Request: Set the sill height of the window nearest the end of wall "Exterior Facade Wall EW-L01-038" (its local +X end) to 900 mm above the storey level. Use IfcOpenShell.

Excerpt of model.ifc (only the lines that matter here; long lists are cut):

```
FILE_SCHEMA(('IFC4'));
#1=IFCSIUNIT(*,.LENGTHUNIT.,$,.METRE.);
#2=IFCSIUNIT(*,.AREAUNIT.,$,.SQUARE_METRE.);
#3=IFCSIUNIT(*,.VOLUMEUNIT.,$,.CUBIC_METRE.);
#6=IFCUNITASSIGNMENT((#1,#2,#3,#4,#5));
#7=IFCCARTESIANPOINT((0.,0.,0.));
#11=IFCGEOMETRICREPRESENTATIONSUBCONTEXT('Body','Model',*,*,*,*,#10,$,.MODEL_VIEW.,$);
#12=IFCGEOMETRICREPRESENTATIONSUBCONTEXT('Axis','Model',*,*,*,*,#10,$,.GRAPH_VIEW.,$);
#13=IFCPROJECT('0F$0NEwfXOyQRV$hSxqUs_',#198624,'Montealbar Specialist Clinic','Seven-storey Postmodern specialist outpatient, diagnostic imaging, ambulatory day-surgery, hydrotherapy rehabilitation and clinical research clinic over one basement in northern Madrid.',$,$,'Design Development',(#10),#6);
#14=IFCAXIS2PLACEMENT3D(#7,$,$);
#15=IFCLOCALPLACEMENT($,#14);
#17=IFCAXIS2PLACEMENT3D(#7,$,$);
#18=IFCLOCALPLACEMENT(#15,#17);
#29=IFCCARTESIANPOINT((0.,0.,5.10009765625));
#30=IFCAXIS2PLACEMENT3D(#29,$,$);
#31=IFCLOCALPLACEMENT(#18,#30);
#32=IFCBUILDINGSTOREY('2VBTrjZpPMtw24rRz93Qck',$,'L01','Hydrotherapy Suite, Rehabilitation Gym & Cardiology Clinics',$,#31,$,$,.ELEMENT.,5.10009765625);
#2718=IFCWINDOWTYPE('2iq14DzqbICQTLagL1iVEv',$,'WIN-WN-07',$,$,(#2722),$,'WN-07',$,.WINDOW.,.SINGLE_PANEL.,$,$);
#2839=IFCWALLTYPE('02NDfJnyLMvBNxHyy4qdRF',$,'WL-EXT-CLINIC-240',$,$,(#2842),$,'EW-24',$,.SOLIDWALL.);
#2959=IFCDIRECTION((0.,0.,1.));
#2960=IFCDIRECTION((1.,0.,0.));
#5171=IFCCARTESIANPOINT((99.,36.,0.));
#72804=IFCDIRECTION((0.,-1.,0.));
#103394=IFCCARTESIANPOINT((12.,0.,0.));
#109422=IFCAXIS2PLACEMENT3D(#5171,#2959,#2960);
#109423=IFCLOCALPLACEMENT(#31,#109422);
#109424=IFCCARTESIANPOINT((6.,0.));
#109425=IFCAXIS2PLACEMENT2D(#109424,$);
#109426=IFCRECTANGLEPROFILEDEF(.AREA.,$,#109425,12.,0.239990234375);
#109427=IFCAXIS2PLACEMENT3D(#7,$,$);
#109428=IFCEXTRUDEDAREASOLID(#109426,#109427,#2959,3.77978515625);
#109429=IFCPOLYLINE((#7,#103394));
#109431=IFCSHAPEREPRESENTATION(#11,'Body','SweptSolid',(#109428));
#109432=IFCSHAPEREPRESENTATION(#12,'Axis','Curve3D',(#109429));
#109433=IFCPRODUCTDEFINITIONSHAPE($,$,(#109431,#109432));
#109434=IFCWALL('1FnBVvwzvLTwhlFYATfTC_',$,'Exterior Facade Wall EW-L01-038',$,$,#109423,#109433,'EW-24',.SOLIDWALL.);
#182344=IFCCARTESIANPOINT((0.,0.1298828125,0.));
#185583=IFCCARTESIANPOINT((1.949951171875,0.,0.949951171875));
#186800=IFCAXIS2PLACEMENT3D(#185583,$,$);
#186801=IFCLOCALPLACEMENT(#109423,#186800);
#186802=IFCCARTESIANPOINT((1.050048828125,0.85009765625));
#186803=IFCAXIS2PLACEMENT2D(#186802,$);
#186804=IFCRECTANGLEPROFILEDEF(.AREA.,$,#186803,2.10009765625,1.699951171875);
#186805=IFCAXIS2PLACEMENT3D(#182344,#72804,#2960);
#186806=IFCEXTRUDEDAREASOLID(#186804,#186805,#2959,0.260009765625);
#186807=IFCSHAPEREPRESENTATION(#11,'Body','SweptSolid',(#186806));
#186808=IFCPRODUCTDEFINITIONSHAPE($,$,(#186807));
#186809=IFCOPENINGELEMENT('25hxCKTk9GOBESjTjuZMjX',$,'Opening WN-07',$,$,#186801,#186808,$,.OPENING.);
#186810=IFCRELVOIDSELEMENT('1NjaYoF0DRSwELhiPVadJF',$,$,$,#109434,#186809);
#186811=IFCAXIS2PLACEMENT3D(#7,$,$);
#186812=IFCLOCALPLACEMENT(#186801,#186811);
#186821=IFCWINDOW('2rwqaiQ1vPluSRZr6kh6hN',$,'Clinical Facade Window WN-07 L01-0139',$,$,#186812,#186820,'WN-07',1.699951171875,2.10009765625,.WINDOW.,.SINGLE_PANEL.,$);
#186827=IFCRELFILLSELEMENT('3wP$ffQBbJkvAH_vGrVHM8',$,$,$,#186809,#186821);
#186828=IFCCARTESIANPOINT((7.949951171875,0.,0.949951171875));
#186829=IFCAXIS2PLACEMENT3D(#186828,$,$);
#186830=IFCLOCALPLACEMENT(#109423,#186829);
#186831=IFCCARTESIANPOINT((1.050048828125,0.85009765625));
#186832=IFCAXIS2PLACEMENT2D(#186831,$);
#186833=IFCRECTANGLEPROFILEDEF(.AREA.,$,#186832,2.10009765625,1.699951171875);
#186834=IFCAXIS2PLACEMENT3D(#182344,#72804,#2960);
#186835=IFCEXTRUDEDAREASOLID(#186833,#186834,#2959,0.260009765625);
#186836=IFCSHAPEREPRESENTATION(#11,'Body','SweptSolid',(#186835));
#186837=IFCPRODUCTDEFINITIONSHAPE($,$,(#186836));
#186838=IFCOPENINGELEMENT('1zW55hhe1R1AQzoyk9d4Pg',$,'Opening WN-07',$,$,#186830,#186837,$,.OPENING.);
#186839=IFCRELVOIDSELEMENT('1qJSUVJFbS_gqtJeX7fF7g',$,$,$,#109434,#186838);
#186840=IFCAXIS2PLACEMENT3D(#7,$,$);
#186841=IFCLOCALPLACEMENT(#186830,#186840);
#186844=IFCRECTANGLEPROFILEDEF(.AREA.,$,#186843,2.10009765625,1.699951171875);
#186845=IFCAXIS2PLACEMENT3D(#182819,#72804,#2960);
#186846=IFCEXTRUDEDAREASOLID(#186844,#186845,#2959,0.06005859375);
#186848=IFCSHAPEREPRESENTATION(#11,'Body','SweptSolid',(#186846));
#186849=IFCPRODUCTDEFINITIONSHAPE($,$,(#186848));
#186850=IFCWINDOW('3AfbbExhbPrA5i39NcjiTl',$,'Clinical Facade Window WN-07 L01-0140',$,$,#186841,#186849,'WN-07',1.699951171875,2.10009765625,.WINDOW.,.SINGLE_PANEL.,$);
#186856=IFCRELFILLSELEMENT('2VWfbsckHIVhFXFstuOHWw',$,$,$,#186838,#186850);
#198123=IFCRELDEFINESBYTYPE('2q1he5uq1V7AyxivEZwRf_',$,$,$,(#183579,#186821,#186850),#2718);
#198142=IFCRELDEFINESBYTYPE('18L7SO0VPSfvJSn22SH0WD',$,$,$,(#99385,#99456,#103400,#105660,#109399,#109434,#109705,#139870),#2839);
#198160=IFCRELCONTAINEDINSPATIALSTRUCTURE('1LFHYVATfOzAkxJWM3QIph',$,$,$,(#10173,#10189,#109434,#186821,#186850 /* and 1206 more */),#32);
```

```python
import numpy as np
import ifcopenshell
import ifcopenshell.api.geometry
import ifcopenshell.geom
import ifcopenshell.util.element
import ifcopenshell.util.placement
import ifcopenshell.util.shape
import ifcopenshell.util.unit

model = ifcopenshell.open("model.ifc")
unit_scale = ifcopenshell.util.unit.calculate_unit_scale(model)

window = model.by_guid("3AfbbExhbPrA5i39NcjiTl")
opening = window.FillsVoids[0].RelatingOpeningElement
storey = ifcopenshell.util.element.get_container(window, ifc_class="IfcBuildingStorey")
level = ifcopenshell.util.placement.get_local_placement(storey.ObjectPlacement)[2, 3]

# The opening's origin need not be at the sill, so measure its lowest point.
shape = ifcopenshell.geom.create_shape(ifcopenshell.geom.settings(), opening)
bottom = ifcopenshell.util.shape.get_shape_bottom_elevation(shape, shape.geometry) / unit_scale
dz = level + 0.9 / unit_scale - bottom

shift = np.array([0.0, 0.0, dz])
# The window is placed relative to its opening, so it follows when the opening moves.
matrix = ifcopenshell.util.placement.get_local_placement(opening.ObjectPlacement)
matrix[:3, 3] += shift
ifcopenshell.api.geometry.edit_object_placement(
    model, product=opening, matrix=matrix, is_si=False, should_transform_children=True
)

print(f"moved by {dz * unit_scale:+.3f} m")

model.write("model_rev.ifc")
```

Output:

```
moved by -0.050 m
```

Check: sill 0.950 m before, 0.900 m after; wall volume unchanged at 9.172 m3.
